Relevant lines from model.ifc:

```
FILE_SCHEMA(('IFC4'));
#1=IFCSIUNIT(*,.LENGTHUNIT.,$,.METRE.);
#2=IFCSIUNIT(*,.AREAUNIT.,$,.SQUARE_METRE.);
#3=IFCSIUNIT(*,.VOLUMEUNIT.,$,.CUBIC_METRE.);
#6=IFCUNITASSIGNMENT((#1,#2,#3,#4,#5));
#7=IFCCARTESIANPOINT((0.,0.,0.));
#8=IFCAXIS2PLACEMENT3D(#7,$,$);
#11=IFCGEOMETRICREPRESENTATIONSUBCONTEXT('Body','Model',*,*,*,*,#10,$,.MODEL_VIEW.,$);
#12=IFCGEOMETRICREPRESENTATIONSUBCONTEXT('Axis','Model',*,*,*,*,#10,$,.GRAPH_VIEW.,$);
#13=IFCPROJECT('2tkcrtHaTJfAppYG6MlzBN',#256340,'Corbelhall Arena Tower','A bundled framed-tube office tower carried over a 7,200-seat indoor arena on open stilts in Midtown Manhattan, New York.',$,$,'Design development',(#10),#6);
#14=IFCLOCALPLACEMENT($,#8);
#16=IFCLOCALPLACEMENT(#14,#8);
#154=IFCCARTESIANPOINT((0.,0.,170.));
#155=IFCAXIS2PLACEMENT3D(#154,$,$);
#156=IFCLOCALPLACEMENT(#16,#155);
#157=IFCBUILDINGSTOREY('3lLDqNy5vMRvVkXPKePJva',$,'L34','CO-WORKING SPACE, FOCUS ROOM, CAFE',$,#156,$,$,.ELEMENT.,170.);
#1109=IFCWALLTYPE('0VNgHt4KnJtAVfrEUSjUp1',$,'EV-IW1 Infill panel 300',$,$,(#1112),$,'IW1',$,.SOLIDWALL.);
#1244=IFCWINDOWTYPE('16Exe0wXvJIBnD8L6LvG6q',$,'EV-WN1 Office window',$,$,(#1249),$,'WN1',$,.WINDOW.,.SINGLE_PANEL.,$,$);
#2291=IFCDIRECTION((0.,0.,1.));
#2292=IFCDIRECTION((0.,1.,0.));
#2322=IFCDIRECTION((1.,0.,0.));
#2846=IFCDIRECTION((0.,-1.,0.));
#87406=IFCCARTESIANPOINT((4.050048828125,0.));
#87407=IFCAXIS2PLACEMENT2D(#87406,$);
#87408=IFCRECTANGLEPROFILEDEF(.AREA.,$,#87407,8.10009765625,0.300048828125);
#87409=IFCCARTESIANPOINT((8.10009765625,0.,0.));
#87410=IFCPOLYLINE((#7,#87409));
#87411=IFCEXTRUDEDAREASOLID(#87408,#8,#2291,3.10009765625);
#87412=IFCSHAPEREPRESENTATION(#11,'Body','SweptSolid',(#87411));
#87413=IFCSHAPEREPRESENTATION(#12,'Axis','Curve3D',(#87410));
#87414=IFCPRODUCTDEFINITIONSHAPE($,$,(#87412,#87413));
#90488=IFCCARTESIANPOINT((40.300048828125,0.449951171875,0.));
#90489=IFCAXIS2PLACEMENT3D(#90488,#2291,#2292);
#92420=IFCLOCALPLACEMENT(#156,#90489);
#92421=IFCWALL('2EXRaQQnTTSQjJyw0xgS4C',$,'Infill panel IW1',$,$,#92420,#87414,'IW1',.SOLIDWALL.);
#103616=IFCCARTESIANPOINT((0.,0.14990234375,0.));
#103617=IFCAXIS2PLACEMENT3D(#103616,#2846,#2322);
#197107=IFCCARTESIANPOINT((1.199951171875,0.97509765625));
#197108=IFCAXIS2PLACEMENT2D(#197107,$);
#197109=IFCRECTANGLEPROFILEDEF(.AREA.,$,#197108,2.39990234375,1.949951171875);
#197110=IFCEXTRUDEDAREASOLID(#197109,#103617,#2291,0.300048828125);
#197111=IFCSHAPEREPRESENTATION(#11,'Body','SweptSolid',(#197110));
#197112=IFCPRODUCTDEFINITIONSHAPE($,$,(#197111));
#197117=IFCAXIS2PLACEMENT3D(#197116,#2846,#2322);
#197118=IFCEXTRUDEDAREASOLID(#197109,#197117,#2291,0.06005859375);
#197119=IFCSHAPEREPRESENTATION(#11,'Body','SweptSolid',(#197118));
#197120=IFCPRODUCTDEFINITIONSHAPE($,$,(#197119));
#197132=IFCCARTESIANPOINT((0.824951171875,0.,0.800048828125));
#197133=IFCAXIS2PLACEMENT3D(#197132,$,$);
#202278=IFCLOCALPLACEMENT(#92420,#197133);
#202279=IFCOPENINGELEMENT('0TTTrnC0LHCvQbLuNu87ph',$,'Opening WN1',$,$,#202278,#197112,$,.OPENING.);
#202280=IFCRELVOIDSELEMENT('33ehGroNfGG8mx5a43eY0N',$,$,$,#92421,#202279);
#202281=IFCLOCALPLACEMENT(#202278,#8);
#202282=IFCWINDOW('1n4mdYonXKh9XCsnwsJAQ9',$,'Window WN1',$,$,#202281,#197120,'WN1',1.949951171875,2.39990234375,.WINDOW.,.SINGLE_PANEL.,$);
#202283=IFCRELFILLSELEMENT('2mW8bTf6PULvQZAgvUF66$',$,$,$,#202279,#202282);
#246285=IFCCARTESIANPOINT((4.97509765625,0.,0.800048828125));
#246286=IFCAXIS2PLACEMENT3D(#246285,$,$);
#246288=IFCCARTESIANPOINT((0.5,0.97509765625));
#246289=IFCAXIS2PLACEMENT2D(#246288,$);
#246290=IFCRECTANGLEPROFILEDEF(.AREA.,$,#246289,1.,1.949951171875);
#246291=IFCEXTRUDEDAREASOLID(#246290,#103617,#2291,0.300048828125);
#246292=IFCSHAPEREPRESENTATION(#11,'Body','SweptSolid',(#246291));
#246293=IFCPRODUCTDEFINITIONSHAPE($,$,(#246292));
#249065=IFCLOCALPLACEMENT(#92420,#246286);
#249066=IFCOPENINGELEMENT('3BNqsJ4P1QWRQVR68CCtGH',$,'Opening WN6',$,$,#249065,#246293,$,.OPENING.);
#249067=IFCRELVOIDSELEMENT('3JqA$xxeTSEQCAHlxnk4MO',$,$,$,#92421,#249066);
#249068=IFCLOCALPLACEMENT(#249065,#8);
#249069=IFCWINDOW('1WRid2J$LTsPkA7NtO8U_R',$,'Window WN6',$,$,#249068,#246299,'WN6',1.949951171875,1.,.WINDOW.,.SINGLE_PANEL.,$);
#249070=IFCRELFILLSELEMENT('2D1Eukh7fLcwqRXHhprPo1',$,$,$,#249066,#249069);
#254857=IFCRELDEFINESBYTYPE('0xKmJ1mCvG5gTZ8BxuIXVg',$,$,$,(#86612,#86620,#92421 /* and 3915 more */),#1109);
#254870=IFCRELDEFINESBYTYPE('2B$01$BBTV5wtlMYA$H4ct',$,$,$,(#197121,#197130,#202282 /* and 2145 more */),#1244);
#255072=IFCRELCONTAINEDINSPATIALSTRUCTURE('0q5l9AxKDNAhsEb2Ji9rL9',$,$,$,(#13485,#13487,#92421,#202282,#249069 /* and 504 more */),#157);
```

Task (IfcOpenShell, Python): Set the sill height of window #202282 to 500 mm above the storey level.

```python
import numpy as np
import ifcopenshell
import ifcopenshell.api.geometry
import ifcopenshell.geom
import ifcopenshell.util.element
import ifcopenshell.util.placement
import ifcopenshell.util.shape
import ifcopenshell.util.unit

model = ifcopenshell.open("model.ifc")
unit_scale = ifcopenshell.util.unit.calculate_unit_scale(model)

window = model.by_guid("1n4mdYonXKh9XCsnwsJAQ9")
opening = window.FillsVoids[0].RelatingOpeningElement
storey = ifcopenshell.util.element.get_container(window, ifc_class="IfcBuildingStorey")
level = ifcopenshell.util.placement.get_local_placement(storey.ObjectPlacement)[2, 3]

# The opening's origin need not be at the sill, so measure its lowest point.
shape = ifcopenshell.geom.create_shape(ifcopenshell.geom.settings(), opening)
bottom = ifcopenshell.util.shape.get_shape_bottom_elevation(shape, shape.geometry) / unit_scale
dz = level + 0.5 - bottom

shift = np.array([0.0, 0.0, dz])
# The window is placed relative to its opening, so it follows when the opening moves.
matrix = ifcopenshell.util.placement.get_local_placement(opening.ObjectPlacement)
matrix[:3, 3] += shift
ifcopenshell.api.geometry.edit_object_placement(
    model, product=opening, matrix=matrix, is_si=False, should_transform_children=True
)

print(f"moved by {dz * unit_scale:+.3f} m")

model.write("model_updated.ifc")
```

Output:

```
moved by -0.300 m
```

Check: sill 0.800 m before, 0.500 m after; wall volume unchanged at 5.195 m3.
